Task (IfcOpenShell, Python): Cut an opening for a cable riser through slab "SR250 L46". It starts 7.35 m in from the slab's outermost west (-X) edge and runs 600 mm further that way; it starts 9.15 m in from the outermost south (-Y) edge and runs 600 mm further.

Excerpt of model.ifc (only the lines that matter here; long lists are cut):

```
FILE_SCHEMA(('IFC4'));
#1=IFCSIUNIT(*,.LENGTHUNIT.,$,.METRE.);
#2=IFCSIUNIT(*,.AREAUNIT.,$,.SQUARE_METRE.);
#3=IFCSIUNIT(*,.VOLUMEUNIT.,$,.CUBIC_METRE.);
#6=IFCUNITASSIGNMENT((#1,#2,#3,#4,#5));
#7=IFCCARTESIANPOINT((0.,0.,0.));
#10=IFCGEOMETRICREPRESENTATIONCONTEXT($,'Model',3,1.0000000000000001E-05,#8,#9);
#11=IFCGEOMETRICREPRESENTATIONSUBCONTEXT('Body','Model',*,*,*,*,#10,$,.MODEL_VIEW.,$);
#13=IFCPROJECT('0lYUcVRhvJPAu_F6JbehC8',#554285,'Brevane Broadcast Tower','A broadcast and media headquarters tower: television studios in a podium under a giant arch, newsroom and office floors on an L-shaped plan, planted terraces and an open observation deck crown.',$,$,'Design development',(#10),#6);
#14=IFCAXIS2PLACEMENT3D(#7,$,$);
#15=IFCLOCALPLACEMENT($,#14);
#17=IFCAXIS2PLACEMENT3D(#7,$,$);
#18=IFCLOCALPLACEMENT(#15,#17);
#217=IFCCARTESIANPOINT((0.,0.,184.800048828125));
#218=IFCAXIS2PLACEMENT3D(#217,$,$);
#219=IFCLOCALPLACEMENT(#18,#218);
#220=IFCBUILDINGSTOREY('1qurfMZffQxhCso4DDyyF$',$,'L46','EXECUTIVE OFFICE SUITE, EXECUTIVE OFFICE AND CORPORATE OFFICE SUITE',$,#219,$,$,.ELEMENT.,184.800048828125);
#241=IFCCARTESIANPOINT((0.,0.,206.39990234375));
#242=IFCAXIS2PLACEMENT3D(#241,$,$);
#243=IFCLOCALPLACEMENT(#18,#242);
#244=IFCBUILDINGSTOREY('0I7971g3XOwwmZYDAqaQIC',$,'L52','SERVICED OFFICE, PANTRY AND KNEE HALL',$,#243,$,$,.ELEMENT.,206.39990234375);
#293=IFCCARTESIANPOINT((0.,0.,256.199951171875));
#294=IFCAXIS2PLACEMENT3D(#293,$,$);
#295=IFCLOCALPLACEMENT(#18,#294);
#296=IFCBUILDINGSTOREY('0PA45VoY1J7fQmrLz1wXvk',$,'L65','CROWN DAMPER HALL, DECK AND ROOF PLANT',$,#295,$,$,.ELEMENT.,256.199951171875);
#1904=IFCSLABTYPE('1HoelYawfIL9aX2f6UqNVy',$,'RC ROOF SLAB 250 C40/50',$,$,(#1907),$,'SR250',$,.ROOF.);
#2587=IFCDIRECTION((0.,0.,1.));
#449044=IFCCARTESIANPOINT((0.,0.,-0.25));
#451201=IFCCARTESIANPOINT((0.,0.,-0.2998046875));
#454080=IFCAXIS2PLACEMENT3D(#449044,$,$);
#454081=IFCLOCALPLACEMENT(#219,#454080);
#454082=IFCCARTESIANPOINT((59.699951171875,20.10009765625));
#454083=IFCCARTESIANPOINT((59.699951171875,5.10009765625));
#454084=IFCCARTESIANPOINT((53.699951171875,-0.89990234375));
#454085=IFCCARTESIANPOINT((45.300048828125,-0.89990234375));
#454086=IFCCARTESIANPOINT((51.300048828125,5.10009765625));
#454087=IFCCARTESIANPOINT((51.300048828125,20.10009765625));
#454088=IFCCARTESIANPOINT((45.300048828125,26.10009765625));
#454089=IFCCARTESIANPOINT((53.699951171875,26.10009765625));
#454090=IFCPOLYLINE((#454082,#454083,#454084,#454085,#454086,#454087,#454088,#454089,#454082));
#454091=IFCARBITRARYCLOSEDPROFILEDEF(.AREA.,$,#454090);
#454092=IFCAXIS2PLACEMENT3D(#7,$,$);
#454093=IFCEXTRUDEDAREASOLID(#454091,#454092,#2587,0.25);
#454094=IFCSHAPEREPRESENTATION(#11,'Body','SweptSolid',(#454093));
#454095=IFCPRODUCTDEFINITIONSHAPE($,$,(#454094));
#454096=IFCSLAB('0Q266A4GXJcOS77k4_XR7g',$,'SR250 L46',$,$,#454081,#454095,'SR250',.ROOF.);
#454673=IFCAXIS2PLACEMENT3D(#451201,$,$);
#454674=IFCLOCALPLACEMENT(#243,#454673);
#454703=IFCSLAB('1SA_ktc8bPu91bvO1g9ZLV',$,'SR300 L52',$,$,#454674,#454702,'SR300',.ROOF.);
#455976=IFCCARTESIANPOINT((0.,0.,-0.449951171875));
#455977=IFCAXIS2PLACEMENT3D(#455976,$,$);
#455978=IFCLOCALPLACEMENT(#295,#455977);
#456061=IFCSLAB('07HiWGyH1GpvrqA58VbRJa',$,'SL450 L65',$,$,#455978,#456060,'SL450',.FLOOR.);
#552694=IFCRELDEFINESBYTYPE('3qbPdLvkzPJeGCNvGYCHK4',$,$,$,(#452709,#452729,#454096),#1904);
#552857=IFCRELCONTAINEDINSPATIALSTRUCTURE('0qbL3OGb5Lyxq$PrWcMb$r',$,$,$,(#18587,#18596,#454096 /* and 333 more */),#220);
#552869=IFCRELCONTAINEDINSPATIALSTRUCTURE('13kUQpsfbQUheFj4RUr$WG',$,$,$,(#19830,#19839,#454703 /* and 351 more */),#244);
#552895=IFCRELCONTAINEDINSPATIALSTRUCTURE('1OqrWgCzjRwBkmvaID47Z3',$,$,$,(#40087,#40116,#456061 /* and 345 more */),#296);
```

```python
import numpy as np
import ifcopenshell
import ifcopenshell.api.feature
import ifcopenshell.api.geometry
import ifcopenshell.api.root
import ifcopenshell.geom
import ifcopenshell.util.placement
import ifcopenshell.util.representation
import ifcopenshell.util.shape
import ifcopenshell.util.unit

model = ifcopenshell.open("model.ifc")
unit_scale = ifcopenshell.util.unit.calculate_unit_scale(model)
settings = ifcopenshell.geom.settings()


def volume(element):
    """Net volume in cubic metres, openings subtracted."""
    shape = ifcopenshell.geom.create_shape(settings, element)
    return ifcopenshell.util.shape.get_volume(shape.geometry)


slab = model.by_guid("0Q266A4GXJcOS77k4_XR7g")
before = volume(slab)

# Extent in the slab's own axes, in metres. The edges named are its -X and -Y sides.
slab_shape = ifcopenshell.geom.create_shape(settings, slab)
vertices = ifcopenshell.util.shape.get_vertices(slab_shape.geometry)
x_min, y_min, bottom = vertices.min(axis=0)
top = vertices[:, 2].max()

opening = ifcopenshell.api.root.create_entity(model, ifc_class="IfcOpeningElement", name="Cable riser opening", predefined_type="OPENING")
context = ifcopenshell.util.representation.get_context(model, "Model", "Body", "MODEL_VIEW")
width, depth = 0.6, 0.6
outline = [(0.0, 0.0), (width, 0.0), (width, depth), (0.0, depth), (0.0, 0.0)]
# Overshoot both faces by 50 mm so the cut is clean.
shape = ifcopenshell.api.geometry.add_slab_representation(
    model, context=context, depth=top - bottom + 0.1, polyline=outline
)
ifcopenshell.api.geometry.assign_representation(model, product=opening, representation=shape)

matrix = ifcopenshell.util.placement.get_local_placement(slab.ObjectPlacement)
matrix[:, 3] = matrix @ np.append(np.array([x_min + 7.35, y_min + 9.15, bottom - 0.05]) / unit_scale, 1.0)
ifcopenshell.api.geometry.edit_object_placement(model, product=opening, matrix=matrix, is_si=False)
ifcopenshell.api.feature.add_feature(model, feature=opening, element=slab)

after = volume(slab)

print(f"slab volume {before:.3f} -> {after:.3f} m3")

model.write("model_rev.ifc")
```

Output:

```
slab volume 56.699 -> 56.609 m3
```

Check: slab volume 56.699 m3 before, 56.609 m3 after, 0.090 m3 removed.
